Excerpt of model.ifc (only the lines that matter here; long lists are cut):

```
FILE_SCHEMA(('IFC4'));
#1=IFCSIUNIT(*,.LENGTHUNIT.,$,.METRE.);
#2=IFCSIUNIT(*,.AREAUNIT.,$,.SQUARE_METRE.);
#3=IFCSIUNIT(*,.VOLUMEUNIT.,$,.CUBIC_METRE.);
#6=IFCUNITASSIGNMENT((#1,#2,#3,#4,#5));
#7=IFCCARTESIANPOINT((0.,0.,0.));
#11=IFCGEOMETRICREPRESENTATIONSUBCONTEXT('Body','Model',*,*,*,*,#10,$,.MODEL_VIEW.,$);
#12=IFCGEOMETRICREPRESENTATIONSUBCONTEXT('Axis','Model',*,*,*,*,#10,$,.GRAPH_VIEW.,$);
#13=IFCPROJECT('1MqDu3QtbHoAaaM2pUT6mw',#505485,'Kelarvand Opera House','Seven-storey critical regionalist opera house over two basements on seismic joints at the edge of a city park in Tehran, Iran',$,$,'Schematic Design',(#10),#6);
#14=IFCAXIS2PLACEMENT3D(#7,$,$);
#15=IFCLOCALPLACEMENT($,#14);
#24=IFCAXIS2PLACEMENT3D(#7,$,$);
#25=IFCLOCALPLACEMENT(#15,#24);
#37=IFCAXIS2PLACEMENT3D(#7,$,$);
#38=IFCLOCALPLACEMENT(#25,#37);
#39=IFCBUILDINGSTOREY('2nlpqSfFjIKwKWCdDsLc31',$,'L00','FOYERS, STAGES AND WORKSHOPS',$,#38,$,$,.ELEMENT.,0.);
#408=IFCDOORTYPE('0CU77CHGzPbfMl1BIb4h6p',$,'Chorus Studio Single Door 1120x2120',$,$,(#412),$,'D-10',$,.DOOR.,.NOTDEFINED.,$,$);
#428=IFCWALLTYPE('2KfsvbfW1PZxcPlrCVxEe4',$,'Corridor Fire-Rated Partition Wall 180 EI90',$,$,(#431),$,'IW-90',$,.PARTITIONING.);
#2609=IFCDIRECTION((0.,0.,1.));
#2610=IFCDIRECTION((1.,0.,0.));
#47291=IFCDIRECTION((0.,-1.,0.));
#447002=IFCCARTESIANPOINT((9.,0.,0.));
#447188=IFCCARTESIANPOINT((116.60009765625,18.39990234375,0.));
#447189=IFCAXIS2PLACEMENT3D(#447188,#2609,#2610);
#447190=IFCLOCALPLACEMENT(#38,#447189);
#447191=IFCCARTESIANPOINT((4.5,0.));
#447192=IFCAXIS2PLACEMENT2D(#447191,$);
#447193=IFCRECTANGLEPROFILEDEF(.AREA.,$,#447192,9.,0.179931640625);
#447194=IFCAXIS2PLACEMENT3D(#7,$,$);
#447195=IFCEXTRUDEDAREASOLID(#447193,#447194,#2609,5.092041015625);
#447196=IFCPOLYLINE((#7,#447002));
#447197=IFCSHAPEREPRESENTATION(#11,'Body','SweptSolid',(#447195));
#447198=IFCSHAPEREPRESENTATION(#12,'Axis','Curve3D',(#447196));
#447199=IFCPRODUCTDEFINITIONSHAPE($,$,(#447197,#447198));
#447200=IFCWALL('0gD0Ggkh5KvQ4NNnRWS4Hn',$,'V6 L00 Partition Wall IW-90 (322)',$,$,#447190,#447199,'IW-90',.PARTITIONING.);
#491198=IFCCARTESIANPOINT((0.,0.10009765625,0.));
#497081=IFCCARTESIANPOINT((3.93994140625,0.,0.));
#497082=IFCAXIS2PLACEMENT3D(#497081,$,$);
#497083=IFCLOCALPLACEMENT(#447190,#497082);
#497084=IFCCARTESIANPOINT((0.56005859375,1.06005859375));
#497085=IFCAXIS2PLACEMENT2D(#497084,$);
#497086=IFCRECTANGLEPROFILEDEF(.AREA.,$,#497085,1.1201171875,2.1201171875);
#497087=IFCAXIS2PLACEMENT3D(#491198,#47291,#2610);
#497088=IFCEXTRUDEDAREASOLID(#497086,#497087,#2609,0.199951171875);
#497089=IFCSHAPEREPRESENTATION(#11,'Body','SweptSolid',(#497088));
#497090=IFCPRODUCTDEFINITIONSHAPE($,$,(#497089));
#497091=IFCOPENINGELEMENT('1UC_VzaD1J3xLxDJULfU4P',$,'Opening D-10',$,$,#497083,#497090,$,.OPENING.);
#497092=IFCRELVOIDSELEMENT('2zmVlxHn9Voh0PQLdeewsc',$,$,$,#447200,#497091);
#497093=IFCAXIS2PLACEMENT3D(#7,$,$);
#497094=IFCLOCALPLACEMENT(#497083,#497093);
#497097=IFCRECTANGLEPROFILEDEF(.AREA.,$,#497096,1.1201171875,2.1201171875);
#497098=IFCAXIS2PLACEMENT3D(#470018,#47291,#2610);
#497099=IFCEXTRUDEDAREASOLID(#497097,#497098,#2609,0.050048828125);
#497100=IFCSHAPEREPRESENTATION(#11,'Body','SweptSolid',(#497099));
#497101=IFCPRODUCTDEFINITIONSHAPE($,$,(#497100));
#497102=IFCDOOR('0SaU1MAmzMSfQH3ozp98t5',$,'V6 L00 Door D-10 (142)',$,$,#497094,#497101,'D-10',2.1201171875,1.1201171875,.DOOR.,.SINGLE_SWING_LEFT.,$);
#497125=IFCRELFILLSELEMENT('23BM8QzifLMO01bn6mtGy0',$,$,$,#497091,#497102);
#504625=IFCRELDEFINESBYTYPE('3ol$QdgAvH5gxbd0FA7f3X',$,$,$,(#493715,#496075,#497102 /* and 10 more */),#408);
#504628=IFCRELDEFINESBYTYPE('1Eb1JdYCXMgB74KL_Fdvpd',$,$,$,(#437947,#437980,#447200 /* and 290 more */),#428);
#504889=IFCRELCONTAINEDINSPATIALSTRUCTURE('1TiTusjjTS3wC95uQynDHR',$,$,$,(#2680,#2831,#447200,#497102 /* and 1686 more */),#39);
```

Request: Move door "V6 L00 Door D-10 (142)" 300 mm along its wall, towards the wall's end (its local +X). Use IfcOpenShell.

```python
import ifcopenshell
import ifcopenshell.api.geometry
import ifcopenshell.util.placement
import ifcopenshell.util.unit

model = ifcopenshell.open("model.ifc")
unit_scale = ifcopenshell.util.unit.calculate_unit_scale(model)

door = model.by_guid("0SaU1MAmzMSfQH3ozp98t5")
opening = door.FillsVoids[0].RelatingOpeningElement
wall = opening.VoidsElements[0].RelatingBuildingElement

wall_matrix = ifcopenshell.util.placement.get_local_placement(wall.ObjectPlacement)
shift = wall_matrix[:3, 0] * 0.3 / unit_scale
before = ifcopenshell.util.placement.get_local_placement(door.ObjectPlacement)[:3, 3].copy()

# The door is placed relative to its opening, so it follows when the opening moves.
matrix = ifcopenshell.util.placement.get_local_placement(opening.ObjectPlacement)
matrix[:3, 3] += shift
ifcopenshell.api.geometry.edit_object_placement(
    model, product=opening, matrix=matrix, is_si=False, should_transform_children=True
)

after = ifcopenshell.util.placement.get_local_placement(door.ObjectPlacement)[:3, 3]
print("door moved by", (after - before).round(3) + 0.0)

model.write("model_rev.ifc")
```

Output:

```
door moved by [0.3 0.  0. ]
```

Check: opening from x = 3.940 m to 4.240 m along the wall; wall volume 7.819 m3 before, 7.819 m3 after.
